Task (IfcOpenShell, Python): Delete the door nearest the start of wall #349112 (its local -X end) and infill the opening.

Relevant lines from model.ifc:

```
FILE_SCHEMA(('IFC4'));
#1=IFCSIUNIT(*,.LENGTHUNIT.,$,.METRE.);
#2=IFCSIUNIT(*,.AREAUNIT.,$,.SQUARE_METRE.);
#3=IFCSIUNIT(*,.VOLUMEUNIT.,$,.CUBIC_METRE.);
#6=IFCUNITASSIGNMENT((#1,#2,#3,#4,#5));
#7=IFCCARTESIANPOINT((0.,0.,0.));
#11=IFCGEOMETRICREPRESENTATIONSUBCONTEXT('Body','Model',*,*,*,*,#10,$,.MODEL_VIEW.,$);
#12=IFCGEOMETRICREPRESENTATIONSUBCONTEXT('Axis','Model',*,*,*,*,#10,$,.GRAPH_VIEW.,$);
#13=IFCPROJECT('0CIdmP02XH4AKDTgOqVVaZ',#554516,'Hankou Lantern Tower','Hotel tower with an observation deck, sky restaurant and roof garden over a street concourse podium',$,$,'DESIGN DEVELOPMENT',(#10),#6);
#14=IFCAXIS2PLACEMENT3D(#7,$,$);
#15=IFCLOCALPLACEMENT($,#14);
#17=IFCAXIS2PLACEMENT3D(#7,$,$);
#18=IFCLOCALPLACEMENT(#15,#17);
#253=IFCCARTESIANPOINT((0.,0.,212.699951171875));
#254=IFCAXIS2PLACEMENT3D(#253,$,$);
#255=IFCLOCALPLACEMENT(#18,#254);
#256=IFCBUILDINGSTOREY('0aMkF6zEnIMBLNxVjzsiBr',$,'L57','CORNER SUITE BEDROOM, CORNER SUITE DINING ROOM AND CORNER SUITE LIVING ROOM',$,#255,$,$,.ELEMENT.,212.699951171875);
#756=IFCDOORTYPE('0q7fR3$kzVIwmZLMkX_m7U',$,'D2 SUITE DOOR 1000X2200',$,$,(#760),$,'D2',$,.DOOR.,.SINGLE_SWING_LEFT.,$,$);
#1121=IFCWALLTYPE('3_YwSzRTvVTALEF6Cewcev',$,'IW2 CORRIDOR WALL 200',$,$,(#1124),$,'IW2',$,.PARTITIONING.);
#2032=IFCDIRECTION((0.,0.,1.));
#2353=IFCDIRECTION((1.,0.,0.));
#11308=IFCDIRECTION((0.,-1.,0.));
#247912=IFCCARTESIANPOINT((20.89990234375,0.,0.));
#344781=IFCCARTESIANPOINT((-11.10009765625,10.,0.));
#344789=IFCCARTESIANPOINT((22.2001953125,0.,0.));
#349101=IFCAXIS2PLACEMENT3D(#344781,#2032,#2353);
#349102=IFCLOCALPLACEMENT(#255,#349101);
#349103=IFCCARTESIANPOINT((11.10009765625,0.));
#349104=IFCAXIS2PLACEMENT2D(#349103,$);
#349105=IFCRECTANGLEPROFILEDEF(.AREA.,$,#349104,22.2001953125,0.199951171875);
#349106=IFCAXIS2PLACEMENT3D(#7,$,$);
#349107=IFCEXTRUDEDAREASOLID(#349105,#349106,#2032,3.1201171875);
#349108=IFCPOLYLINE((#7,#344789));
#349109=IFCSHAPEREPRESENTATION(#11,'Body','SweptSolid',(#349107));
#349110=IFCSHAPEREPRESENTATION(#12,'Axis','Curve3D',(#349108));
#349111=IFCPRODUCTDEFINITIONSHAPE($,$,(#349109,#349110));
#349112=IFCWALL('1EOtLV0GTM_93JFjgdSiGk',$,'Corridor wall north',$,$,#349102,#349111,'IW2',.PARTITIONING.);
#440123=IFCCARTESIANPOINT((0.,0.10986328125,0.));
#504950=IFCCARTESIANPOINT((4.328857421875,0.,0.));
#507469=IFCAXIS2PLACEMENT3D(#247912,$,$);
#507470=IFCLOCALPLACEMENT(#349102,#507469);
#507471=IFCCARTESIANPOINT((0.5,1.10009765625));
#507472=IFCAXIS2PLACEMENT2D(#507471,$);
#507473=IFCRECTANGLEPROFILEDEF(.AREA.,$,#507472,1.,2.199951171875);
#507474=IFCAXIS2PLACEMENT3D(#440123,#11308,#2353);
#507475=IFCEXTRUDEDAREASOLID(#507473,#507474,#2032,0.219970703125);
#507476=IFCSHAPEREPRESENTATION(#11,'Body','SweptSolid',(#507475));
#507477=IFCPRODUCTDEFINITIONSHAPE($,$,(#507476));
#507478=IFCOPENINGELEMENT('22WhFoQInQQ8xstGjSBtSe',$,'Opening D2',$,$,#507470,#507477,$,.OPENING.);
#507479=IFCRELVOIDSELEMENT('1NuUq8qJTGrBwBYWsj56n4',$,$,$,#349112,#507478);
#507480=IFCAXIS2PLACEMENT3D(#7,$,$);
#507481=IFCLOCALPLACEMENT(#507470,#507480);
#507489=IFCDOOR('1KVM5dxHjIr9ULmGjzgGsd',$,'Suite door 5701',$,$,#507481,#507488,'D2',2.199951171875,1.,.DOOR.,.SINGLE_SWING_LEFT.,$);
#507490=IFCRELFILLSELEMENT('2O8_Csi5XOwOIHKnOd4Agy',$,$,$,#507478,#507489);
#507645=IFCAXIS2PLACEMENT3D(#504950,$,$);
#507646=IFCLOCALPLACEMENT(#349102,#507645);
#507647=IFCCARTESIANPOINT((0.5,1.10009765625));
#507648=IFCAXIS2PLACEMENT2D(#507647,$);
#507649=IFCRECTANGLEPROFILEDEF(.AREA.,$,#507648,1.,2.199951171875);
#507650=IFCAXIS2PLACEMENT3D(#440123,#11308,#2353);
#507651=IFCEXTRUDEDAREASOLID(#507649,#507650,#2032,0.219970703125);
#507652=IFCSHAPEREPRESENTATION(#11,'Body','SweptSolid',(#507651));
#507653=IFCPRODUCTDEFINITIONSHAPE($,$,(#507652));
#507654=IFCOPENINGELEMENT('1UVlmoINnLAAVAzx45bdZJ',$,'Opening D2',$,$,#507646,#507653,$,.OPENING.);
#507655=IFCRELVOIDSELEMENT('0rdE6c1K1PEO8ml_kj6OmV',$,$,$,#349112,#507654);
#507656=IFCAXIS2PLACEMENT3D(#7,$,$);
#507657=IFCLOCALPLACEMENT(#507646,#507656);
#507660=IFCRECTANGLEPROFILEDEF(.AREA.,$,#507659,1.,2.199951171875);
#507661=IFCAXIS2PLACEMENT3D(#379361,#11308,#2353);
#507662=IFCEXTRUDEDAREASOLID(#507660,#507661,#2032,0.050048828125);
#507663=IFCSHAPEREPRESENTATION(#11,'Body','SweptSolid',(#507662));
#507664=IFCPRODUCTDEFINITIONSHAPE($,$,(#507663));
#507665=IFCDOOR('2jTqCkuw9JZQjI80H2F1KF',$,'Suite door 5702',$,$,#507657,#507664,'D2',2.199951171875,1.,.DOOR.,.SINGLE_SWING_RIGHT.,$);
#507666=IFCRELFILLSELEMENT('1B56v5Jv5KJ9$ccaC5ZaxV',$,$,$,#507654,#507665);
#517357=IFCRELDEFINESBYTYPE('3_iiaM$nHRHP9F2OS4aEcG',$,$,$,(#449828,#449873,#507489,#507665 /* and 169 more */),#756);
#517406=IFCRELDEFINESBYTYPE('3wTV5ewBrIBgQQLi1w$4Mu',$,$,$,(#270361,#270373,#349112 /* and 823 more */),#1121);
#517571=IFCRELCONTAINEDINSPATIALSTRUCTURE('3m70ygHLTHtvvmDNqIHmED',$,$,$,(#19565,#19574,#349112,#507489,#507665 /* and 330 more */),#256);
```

```python
import ifcopenshell
import ifcopenshell.api.feature
import ifcopenshell.api.root
import ifcopenshell.geom
import ifcopenshell.util.shape

model = ifcopenshell.open("model.ifc")
settings = ifcopenshell.geom.settings()


def volume(element):
    """Net volume in cubic metres, openings subtracted."""
    shape = ifcopenshell.geom.create_shape(settings, element)
    return ifcopenshell.util.shape.get_volume(shape.geometry)


door = model.by_guid("2jTqCkuw9JZQjI80H2F1KF")
opening = door.FillsVoids[0].RelatingOpeningElement
wall = opening.VoidsElements[0].RelatingBuildingElement
before = volume(wall)

ifcopenshell.api.root.remove_product(model, product=door)
ifcopenshell.api.feature.remove_feature(model, feature=opening)

after = volume(wall)

print(f"wall volume {before:.3f} -> {after:.3f} m3")

model.write("model_edited.ifc")
```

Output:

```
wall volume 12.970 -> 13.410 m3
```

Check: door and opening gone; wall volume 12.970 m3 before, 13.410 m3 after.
